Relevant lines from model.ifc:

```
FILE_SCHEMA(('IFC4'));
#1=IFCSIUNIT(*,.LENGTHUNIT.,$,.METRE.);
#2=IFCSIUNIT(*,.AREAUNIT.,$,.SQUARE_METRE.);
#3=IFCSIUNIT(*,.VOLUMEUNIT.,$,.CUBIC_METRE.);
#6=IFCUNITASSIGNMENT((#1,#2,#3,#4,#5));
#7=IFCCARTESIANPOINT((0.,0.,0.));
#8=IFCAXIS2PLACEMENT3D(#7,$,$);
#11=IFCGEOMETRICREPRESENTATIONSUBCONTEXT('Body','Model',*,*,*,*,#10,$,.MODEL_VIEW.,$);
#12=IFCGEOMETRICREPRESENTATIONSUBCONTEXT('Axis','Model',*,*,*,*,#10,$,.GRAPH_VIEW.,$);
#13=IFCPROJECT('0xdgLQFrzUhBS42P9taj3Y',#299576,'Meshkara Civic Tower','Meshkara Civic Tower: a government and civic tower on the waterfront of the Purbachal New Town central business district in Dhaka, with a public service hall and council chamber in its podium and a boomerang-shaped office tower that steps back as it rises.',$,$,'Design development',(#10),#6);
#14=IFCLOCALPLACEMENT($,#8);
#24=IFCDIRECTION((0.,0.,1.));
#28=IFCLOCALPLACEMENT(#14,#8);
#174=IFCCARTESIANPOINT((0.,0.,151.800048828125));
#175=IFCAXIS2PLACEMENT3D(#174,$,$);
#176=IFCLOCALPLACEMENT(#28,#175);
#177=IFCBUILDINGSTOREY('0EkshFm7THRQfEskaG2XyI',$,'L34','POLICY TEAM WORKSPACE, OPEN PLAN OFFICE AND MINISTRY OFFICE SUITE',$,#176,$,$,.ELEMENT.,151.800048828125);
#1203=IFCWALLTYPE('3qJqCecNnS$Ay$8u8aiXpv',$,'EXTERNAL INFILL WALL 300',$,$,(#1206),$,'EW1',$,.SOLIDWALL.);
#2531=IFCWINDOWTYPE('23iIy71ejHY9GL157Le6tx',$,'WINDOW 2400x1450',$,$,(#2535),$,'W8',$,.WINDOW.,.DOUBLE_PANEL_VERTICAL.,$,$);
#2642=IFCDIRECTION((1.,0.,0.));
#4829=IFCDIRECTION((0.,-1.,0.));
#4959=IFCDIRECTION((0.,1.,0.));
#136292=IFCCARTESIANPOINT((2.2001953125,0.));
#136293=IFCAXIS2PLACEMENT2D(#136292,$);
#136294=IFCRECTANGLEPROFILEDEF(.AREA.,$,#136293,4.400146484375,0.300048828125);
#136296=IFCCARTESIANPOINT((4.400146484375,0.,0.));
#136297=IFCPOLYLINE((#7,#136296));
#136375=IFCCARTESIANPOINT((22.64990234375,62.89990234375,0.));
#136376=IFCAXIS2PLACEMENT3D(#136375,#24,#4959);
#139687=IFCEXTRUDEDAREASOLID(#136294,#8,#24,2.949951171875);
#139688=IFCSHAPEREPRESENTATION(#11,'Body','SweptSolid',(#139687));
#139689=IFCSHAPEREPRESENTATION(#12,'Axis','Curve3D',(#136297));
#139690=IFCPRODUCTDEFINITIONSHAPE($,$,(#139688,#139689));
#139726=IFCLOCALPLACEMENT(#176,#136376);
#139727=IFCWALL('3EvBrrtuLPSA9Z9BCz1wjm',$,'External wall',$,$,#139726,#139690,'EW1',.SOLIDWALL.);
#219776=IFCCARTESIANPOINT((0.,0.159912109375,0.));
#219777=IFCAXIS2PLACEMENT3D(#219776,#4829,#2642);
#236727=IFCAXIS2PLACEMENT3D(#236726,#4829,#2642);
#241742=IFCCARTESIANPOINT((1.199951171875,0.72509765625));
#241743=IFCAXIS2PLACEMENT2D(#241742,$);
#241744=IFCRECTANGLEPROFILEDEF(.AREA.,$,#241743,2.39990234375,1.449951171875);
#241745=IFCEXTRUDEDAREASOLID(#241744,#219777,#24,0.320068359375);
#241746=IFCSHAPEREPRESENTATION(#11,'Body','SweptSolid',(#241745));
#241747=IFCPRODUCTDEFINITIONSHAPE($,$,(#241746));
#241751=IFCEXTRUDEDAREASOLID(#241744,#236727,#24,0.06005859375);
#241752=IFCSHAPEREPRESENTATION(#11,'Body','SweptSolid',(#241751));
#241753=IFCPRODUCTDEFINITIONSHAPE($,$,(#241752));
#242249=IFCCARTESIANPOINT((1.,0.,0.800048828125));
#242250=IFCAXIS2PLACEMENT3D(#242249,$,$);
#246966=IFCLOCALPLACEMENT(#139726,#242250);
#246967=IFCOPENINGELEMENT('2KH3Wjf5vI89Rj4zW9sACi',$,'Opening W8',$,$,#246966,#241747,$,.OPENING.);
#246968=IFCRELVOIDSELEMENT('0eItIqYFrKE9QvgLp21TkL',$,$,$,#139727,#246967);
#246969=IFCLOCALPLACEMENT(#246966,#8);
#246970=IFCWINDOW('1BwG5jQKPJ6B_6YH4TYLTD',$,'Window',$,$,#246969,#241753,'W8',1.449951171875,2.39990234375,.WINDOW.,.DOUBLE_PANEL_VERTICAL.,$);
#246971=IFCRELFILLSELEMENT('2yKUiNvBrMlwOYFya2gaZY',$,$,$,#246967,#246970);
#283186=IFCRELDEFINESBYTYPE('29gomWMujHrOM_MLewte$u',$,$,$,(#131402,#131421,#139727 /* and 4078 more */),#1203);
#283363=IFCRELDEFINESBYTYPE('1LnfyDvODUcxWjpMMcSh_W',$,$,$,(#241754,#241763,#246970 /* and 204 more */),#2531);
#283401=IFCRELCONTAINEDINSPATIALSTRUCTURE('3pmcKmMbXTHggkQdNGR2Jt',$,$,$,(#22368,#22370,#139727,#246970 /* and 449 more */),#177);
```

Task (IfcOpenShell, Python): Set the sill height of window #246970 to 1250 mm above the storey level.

```python
import numpy as np
import ifcopenshell
import ifcopenshell.api.geometry
import ifcopenshell.geom
import ifcopenshell.util.element
import ifcopenshell.util.placement
import ifcopenshell.util.shape
import ifcopenshell.util.unit

model = ifcopenshell.open("model.ifc")
unit_scale = ifcopenshell.util.unit.calculate_unit_scale(model)

window = model.by_id(246970)
opening = window.FillsVoids[0].RelatingOpeningElement
storey = ifcopenshell.util.element.get_container(window, ifc_class="IfcBuildingStorey")
level = ifcopenshell.util.placement.get_local_placement(storey.ObjectPlacement)[2, 3]

# The opening's origin need not be at the sill, so measure its lowest point.
shape = ifcopenshell.geom.create_shape(ifcopenshell.geom.settings(), opening)
bottom = ifcopenshell.util.shape.get_shape_bottom_elevation(shape, shape.geometry) / unit_scale
dz = level + 1.25 / unit_scale - bottom

shift = np.array([0.0, 0.0, dz])
# The window is placed relative to its opening, so it follows when the opening moves.
matrix = ifcopenshell.util.placement.get_local_placement(opening.ObjectPlacement)
matrix[:3, 3] += shift
ifcopenshell.api.geometry.edit_object_placement(
    model, product=opening, matrix=matrix, is_si=False, should_transform_children=True
)

print(f"moved by {dz * unit_scale:+.3f} m")

model.write("model_v2.ifc")
```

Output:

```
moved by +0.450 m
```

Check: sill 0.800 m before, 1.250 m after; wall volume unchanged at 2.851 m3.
